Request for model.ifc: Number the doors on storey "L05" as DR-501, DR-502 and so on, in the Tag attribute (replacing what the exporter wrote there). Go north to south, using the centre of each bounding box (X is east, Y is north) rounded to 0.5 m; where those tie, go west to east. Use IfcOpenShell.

First a look at what the model holds.

```python
import ifcopenshell
import ifcopenshell.util.element
import ifcopenshell.util.placement

model = ifcopenshell.open("model.ifc")
print(model.schema)
storey = next(s for s in model.by_type("IfcBuildingStorey") if s.Name == "L05")
doors = [e for e in ifcopenshell.util.element.get_decomposition(storey) if e.is_a("IfcDoor")]
for e in sorted(doors, key=lambda e: e.id()):
    origin = ifcopenshell.util.placement.get_local_placement(e.ObjectPlacement)[:3, 3]
    print(e.id(), e.Tag, e.Name, origin.round(2) + 0.0, sep=" | ")
```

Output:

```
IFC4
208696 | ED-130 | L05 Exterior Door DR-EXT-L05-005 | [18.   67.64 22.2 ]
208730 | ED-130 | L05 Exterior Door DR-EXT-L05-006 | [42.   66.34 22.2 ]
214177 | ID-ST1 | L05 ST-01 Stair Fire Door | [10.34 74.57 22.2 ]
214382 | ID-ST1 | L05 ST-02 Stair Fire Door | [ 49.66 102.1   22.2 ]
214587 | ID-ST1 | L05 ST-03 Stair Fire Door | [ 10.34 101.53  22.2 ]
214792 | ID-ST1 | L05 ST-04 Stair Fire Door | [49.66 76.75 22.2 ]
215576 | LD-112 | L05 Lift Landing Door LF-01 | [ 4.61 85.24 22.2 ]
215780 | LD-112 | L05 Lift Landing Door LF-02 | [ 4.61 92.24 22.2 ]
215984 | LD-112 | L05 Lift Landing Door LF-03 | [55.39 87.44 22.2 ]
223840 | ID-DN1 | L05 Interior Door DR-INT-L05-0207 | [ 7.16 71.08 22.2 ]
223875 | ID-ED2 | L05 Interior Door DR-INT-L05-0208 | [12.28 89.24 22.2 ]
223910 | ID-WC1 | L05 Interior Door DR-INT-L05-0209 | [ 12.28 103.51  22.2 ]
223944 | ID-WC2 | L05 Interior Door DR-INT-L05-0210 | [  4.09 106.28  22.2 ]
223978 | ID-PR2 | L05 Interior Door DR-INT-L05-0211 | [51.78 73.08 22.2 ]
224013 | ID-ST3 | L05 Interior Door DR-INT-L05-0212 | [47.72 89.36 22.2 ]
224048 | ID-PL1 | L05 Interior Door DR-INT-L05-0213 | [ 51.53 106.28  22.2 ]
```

```python
import ifcopenshell
import ifcopenshell.geom
import ifcopenshell.util.element
import ifcopenshell.util.shape

model = ifcopenshell.open("model.ifc")
settings = ifcopenshell.geom.settings()
settings.set("use-world-coords", True)


def centre(element):
    shape = ifcopenshell.geom.create_shape(settings, element)
    return ifcopenshell.util.shape.get_bbox_centroid(shape.geometry)


storey = next(s for s in model.by_type("IfcBuildingStorey") if s.Name == "L05")
doors = [e for e in ifcopenshell.util.element.get_decomposition(storey) if e.is_a("IfcDoor")]

# Insertion points can sit at a corner or the storey origin, so sort by the geometry (in metres).
centres = {e: centre(e) for e in doors}
doors.sort(key=lambda e: (-round(centres[e][1] / 0.5), centres[e][0]))

for i, e in enumerate(doors, start=1):
    number = f"DR-5{i:02d}"
    e.Tag = number
    print(e.id(), number)

model.write("model_rev.ifc")
```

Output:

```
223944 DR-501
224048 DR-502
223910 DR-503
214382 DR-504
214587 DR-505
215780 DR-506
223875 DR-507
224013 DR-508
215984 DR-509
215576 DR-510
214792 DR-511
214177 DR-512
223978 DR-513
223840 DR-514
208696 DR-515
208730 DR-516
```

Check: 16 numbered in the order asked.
